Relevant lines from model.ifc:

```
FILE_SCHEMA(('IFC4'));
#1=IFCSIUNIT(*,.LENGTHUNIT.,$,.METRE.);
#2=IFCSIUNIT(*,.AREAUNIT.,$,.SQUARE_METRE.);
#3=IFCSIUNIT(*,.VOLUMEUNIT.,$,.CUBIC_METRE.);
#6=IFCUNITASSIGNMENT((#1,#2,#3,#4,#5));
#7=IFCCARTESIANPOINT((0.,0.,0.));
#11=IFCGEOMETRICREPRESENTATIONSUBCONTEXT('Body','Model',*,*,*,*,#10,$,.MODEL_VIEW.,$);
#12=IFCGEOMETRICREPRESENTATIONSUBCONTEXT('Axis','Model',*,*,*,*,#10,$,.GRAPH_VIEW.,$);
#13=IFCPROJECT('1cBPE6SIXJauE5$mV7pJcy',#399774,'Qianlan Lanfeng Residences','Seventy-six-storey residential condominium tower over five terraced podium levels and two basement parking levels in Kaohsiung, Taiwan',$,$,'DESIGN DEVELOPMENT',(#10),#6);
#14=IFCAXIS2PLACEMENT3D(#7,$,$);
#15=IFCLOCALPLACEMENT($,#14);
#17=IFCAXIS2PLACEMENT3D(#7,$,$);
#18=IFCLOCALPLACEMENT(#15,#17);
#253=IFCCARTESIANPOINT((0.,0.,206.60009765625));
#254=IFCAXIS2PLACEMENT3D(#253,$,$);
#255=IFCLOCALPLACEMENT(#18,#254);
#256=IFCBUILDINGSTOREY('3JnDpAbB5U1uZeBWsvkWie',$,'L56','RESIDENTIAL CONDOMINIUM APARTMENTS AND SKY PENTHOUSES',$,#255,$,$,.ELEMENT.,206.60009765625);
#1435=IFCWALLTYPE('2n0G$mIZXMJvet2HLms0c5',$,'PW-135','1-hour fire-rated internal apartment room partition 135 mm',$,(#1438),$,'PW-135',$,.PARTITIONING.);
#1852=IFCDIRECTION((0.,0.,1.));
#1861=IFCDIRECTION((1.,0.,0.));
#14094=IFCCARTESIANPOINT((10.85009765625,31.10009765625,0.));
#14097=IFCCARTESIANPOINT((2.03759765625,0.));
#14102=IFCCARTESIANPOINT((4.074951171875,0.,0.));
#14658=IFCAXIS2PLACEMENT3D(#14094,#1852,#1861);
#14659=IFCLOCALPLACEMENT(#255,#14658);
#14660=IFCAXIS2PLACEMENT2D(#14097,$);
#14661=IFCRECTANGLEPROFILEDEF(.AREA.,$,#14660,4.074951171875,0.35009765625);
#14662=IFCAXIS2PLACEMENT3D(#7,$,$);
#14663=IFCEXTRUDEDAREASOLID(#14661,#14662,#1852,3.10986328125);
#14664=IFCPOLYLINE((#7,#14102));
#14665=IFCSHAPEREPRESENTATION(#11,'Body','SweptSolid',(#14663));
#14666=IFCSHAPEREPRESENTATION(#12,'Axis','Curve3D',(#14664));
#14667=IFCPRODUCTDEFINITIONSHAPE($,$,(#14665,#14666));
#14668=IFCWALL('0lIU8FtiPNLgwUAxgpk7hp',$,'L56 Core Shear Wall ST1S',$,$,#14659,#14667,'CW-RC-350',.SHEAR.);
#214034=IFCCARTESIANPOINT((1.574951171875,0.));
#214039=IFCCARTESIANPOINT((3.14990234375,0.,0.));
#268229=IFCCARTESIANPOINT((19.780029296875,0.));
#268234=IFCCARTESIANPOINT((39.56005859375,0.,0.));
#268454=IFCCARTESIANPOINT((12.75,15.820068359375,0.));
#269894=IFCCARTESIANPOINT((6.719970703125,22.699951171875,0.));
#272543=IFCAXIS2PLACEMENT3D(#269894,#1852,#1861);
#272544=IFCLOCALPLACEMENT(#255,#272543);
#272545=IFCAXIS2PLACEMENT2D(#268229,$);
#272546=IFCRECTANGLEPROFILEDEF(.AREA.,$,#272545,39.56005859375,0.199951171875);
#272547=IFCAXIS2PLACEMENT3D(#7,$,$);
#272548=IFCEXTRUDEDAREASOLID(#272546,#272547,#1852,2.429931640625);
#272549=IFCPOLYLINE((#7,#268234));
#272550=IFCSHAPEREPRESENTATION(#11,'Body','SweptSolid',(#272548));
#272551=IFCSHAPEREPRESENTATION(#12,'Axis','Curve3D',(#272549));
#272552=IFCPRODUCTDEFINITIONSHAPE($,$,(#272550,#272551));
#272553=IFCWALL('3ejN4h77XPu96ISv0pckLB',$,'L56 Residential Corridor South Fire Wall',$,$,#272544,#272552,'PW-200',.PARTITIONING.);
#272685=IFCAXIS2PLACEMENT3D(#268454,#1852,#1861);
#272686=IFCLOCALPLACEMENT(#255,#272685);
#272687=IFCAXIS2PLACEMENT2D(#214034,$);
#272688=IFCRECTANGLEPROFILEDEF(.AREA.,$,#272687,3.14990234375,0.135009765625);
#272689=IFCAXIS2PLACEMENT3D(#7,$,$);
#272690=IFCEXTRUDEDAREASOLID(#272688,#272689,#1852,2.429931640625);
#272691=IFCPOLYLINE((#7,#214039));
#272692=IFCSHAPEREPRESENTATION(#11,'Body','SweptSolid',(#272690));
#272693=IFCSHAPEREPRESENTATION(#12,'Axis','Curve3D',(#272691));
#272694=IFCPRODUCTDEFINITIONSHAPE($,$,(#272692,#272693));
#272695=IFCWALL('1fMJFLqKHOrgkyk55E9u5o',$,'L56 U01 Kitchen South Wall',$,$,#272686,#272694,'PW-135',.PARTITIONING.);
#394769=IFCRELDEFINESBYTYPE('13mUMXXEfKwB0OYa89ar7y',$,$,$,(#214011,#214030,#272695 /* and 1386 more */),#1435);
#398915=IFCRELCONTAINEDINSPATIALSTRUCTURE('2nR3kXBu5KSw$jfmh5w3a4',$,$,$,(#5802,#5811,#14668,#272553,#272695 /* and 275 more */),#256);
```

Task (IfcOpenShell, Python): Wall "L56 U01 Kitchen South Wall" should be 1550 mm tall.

```python
import ifcopenshell
import ifcopenshell.geom
import ifcopenshell.util.representation
import ifcopenshell.util.shape
import ifcopenshell.util.unit

model = ifcopenshell.open("model.ifc")
unit_scale = ifcopenshell.util.unit.calculate_unit_scale(model)
settings = ifcopenshell.geom.settings()


def volume(element):
    """Net volume in cubic metres, openings subtracted."""
    shape = ifcopenshell.geom.create_shape(settings, element)
    return ifcopenshell.util.shape.get_volume(shape.geometry)


wall = model.by_guid("1fMJFLqKHOrgkyk55E9u5o")
before = volume(wall)

body = ifcopenshell.util.representation.get_representation(wall, "Model", "Body")
solid = body.Items[0]
old_height = solid.Depth
solid.Depth = 1.55 / unit_scale
after = volume(wall)

print(f"height {old_height:g} -> {solid.Depth:g}, volume {before:.3f} -> {after:.3f} m3")

model.write("model_edited.ifc")
```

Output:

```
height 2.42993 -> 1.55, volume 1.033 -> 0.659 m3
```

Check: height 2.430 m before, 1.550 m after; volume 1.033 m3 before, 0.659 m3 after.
